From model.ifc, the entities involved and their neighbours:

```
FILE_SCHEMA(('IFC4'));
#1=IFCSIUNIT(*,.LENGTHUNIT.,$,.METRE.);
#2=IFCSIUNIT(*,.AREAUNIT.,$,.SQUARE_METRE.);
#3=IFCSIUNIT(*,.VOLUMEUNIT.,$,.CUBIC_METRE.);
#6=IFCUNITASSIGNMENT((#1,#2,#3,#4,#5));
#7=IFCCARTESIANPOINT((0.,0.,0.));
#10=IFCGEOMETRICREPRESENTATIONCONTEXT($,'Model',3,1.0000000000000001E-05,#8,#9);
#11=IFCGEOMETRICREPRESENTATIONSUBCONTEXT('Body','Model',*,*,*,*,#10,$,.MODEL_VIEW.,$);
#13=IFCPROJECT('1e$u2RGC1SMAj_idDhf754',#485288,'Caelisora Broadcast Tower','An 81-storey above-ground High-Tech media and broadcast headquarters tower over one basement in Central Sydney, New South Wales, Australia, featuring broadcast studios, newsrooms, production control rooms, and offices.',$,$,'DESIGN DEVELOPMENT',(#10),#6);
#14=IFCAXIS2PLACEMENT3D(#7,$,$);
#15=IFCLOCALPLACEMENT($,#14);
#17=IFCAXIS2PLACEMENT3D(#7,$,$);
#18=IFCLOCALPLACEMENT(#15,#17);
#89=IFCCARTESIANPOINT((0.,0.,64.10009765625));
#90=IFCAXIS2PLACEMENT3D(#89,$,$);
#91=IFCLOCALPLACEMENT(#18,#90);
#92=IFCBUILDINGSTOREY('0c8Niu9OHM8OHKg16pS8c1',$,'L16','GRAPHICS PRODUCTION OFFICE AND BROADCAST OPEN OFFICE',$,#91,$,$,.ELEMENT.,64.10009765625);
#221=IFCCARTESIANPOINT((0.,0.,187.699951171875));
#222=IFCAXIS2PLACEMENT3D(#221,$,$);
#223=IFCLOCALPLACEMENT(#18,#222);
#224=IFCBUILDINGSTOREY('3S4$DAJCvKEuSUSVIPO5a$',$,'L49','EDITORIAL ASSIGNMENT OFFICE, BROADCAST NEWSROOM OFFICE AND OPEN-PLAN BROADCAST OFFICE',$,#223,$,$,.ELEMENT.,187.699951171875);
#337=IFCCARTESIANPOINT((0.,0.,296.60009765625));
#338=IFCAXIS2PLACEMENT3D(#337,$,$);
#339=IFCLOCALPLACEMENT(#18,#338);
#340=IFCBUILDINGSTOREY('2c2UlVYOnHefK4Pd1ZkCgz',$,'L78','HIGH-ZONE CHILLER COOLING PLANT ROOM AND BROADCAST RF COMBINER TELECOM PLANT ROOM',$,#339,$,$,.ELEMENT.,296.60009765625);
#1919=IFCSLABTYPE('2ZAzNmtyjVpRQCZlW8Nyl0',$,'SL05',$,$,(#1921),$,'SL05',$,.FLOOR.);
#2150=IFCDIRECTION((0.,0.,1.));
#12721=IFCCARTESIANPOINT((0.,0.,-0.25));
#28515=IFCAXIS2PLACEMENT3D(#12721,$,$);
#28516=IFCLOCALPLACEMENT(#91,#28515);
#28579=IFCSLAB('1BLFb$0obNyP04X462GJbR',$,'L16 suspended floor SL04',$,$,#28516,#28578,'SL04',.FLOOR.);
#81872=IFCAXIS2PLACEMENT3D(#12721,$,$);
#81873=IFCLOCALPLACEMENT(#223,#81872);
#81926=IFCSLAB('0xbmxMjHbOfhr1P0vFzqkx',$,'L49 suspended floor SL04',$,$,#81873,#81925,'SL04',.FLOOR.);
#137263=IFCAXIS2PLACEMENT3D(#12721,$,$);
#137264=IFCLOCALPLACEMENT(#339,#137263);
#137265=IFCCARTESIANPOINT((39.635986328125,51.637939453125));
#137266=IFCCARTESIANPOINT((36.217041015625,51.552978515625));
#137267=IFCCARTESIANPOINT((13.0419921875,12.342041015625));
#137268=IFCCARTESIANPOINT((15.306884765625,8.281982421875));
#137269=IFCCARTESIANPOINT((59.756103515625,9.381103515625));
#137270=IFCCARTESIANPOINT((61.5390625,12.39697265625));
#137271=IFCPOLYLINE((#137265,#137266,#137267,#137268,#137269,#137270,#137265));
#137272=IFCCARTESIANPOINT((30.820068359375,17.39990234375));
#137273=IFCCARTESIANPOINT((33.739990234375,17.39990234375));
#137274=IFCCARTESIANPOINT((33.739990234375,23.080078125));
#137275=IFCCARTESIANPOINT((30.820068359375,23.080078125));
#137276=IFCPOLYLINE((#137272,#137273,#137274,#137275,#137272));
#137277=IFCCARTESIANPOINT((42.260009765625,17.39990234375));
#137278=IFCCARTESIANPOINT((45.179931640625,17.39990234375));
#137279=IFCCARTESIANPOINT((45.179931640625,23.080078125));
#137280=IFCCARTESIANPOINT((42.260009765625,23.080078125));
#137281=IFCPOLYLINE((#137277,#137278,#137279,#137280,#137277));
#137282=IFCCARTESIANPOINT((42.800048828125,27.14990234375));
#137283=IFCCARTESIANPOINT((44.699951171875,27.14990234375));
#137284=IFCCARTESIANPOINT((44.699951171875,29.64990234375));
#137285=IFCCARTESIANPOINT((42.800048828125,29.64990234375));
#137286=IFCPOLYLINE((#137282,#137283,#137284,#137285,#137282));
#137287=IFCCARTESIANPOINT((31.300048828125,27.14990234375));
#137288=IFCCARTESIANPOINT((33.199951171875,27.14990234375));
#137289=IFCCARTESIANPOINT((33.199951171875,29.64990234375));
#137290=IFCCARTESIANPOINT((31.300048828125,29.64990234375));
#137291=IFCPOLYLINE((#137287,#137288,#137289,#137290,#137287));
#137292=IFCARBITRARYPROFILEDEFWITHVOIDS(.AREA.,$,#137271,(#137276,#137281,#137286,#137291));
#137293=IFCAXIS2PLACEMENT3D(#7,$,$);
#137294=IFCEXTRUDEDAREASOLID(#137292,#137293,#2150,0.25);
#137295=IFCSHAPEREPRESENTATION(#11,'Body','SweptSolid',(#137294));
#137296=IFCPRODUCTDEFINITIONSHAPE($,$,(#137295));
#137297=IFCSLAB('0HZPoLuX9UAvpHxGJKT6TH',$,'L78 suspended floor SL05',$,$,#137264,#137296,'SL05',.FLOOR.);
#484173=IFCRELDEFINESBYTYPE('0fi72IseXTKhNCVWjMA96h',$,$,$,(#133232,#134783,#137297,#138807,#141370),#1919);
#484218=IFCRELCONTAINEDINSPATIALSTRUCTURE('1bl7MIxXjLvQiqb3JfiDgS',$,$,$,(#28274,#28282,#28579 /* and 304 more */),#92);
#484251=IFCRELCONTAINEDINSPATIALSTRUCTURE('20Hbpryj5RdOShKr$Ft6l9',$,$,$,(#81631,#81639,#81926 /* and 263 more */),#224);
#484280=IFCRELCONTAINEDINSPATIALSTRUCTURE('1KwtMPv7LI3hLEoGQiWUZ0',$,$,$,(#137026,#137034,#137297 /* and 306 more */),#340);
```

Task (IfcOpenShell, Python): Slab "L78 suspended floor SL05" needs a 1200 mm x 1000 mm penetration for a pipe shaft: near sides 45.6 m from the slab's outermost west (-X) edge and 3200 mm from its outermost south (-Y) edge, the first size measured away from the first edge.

```python
import numpy as np
import ifcopenshell
import ifcopenshell.api.feature
import ifcopenshell.api.geometry
import ifcopenshell.api.root
import ifcopenshell.geom
import ifcopenshell.util.placement
import ifcopenshell.util.representation
import ifcopenshell.util.shape
import ifcopenshell.util.unit

model = ifcopenshell.open("model.ifc")
unit_scale = ifcopenshell.util.unit.calculate_unit_scale(model)
settings = ifcopenshell.geom.settings()


def volume(element):
    """Net volume in cubic metres, openings subtracted."""
    shape = ifcopenshell.geom.create_shape(settings, element)
    return ifcopenshell.util.shape.get_volume(shape.geometry)


slab = model.by_id(137297)
before = volume(slab)

# Extent in the slab's own axes, in metres. The edges named are its -X and -Y sides.
slab_shape = ifcopenshell.geom.create_shape(settings, slab)
vertices = ifcopenshell.util.shape.get_vertices(slab_shape.geometry)
x_min, y_min, bottom = vertices.min(axis=0)
top = vertices[:, 2].max()

opening = ifcopenshell.api.root.create_entity(model, ifc_class="IfcOpeningElement", name="Pipe shaft opening", predefined_type="OPENING")
context = ifcopenshell.util.representation.get_context(model, "Model", "Body", "MODEL_VIEW")
width, depth = 1.2, 1
outline = [(0.0, 0.0), (width, 0.0), (width, depth), (0.0, depth), (0.0, 0.0)]
# Overshoot both faces by 50 mm so the cut is clean.
shape = ifcopenshell.api.geometry.add_slab_representation(
    model, context=context, depth=top - bottom + 0.1, polyline=outline
)
ifcopenshell.api.geometry.assign_representation(model, product=opening, representation=shape)

matrix = ifcopenshell.util.placement.get_local_placement(slab.ObjectPlacement)
matrix[:, 3] = matrix @ np.append(np.array([x_min + 45.6, y_min + 3.2, bottom - 0.05]) / unit_scale, 1.0)
ifcopenshell.api.geometry.edit_object_placement(model, product=opening, matrix=matrix, is_si=False)
ifcopenshell.api.feature.add_feature(model, feature=opening, element=slab)

after = volume(slab)

print(f"slab volume {before:.3f} -> {after:.3f} m3")

model.write("model-out.ifc")
```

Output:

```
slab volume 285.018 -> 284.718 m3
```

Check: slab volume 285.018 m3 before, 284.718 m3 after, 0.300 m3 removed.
